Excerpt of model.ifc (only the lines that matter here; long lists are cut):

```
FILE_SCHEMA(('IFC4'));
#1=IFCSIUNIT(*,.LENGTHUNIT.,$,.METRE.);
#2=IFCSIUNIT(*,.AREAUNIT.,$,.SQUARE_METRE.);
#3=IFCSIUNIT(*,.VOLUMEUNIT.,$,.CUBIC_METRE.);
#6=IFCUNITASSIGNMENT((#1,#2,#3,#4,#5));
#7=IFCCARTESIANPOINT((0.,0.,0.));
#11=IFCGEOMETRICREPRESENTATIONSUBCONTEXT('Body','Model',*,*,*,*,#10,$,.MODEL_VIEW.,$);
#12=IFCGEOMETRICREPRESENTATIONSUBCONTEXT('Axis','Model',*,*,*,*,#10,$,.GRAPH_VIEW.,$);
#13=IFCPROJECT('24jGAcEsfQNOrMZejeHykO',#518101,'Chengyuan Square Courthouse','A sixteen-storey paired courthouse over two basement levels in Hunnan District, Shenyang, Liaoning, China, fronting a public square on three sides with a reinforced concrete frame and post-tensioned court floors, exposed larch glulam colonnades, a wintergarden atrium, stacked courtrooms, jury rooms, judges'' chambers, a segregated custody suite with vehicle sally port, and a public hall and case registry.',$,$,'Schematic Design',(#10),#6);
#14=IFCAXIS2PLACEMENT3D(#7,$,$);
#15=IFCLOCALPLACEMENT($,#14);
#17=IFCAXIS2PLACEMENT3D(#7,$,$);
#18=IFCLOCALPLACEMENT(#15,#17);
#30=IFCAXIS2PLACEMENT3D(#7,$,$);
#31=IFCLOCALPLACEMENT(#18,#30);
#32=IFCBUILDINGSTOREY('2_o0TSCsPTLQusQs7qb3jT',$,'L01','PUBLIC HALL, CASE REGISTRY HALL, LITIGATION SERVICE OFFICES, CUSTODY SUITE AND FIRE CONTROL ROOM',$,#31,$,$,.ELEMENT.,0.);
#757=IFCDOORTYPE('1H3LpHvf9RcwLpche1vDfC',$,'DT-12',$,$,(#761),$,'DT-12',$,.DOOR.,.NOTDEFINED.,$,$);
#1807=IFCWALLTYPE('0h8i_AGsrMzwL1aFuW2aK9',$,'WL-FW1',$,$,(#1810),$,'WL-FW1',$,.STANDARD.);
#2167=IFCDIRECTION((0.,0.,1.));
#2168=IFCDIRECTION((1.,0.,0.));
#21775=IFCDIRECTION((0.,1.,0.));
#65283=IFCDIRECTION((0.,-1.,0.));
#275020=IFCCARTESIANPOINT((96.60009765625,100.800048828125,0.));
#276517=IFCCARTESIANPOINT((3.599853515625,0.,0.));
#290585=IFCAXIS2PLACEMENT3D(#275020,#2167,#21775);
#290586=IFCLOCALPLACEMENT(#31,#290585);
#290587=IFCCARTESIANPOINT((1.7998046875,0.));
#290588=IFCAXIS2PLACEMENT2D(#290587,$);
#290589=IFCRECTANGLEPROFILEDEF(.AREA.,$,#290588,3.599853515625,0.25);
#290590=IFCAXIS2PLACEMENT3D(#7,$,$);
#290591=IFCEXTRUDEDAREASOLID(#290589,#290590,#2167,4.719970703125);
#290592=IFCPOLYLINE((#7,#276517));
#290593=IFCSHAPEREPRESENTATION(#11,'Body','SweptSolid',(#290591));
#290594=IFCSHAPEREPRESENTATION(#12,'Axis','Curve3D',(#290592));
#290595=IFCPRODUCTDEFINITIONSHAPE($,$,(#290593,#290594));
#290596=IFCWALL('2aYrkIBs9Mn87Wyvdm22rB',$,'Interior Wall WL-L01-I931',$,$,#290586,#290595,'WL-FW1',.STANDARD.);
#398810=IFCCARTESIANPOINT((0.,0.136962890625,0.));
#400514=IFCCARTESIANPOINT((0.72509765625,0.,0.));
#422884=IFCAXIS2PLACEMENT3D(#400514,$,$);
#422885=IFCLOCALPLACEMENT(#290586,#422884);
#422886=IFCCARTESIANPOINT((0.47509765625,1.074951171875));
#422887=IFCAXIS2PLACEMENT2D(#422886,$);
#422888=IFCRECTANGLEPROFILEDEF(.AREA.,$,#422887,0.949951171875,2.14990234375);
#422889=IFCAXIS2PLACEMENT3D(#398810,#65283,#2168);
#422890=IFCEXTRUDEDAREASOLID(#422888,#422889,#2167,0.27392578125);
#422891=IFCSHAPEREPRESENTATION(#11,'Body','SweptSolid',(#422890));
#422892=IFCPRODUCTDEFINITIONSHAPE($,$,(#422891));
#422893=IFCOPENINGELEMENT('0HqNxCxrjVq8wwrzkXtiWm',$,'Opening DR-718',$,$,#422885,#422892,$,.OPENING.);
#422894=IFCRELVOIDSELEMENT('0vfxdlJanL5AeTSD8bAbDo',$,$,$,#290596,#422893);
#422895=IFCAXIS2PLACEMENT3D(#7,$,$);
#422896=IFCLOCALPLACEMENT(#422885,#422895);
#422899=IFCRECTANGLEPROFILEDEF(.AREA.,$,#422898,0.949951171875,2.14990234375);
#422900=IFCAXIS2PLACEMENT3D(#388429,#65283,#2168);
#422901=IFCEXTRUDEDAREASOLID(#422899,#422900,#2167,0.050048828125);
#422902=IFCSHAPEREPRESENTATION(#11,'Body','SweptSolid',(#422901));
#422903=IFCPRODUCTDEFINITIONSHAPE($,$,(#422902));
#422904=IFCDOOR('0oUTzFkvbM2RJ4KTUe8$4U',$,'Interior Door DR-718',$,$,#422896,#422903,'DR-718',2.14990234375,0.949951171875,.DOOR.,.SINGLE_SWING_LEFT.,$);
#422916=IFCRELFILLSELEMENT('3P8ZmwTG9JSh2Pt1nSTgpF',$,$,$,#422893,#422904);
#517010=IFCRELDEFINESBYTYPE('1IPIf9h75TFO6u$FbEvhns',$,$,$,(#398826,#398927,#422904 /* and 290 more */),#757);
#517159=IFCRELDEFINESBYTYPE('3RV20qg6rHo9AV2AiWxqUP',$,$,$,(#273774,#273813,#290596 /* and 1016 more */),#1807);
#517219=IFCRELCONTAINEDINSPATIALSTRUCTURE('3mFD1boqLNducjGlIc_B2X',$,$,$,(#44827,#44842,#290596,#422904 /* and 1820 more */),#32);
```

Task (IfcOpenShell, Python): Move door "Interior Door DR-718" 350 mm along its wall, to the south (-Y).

```python
import ifcopenshell
import ifcopenshell.api.geometry
import ifcopenshell.util.placement
import ifcopenshell.util.unit

model = ifcopenshell.open("model.ifc")
unit_scale = ifcopenshell.util.unit.calculate_unit_scale(model)

door = model.by_guid("0oUTzFkvbM2RJ4KTUe8$4U")
opening = door.FillsVoids[0].RelatingOpeningElement
wall = opening.VoidsElements[0].RelatingBuildingElement

wall_matrix = ifcopenshell.util.placement.get_local_placement(wall.ObjectPlacement)
shift = wall_matrix[:3, 0] * -0.35 / unit_scale
before = ifcopenshell.util.placement.get_local_placement(door.ObjectPlacement)[:3, 3].copy()

# The door is placed relative to its opening, so it follows when the opening moves.
matrix = ifcopenshell.util.placement.get_local_placement(opening.ObjectPlacement)
matrix[:3, 3] += shift
ifcopenshell.api.geometry.edit_object_placement(
    model, product=opening, matrix=matrix, is_si=False, should_transform_children=True
)

after = ifcopenshell.util.placement.get_local_placement(door.ObjectPlacement)[:3, 3]
print("door moved by", (after - before).round(3) + 0.0)

model.write("model-out.ifc")
```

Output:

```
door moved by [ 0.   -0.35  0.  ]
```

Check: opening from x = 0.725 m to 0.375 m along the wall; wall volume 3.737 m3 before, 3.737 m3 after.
